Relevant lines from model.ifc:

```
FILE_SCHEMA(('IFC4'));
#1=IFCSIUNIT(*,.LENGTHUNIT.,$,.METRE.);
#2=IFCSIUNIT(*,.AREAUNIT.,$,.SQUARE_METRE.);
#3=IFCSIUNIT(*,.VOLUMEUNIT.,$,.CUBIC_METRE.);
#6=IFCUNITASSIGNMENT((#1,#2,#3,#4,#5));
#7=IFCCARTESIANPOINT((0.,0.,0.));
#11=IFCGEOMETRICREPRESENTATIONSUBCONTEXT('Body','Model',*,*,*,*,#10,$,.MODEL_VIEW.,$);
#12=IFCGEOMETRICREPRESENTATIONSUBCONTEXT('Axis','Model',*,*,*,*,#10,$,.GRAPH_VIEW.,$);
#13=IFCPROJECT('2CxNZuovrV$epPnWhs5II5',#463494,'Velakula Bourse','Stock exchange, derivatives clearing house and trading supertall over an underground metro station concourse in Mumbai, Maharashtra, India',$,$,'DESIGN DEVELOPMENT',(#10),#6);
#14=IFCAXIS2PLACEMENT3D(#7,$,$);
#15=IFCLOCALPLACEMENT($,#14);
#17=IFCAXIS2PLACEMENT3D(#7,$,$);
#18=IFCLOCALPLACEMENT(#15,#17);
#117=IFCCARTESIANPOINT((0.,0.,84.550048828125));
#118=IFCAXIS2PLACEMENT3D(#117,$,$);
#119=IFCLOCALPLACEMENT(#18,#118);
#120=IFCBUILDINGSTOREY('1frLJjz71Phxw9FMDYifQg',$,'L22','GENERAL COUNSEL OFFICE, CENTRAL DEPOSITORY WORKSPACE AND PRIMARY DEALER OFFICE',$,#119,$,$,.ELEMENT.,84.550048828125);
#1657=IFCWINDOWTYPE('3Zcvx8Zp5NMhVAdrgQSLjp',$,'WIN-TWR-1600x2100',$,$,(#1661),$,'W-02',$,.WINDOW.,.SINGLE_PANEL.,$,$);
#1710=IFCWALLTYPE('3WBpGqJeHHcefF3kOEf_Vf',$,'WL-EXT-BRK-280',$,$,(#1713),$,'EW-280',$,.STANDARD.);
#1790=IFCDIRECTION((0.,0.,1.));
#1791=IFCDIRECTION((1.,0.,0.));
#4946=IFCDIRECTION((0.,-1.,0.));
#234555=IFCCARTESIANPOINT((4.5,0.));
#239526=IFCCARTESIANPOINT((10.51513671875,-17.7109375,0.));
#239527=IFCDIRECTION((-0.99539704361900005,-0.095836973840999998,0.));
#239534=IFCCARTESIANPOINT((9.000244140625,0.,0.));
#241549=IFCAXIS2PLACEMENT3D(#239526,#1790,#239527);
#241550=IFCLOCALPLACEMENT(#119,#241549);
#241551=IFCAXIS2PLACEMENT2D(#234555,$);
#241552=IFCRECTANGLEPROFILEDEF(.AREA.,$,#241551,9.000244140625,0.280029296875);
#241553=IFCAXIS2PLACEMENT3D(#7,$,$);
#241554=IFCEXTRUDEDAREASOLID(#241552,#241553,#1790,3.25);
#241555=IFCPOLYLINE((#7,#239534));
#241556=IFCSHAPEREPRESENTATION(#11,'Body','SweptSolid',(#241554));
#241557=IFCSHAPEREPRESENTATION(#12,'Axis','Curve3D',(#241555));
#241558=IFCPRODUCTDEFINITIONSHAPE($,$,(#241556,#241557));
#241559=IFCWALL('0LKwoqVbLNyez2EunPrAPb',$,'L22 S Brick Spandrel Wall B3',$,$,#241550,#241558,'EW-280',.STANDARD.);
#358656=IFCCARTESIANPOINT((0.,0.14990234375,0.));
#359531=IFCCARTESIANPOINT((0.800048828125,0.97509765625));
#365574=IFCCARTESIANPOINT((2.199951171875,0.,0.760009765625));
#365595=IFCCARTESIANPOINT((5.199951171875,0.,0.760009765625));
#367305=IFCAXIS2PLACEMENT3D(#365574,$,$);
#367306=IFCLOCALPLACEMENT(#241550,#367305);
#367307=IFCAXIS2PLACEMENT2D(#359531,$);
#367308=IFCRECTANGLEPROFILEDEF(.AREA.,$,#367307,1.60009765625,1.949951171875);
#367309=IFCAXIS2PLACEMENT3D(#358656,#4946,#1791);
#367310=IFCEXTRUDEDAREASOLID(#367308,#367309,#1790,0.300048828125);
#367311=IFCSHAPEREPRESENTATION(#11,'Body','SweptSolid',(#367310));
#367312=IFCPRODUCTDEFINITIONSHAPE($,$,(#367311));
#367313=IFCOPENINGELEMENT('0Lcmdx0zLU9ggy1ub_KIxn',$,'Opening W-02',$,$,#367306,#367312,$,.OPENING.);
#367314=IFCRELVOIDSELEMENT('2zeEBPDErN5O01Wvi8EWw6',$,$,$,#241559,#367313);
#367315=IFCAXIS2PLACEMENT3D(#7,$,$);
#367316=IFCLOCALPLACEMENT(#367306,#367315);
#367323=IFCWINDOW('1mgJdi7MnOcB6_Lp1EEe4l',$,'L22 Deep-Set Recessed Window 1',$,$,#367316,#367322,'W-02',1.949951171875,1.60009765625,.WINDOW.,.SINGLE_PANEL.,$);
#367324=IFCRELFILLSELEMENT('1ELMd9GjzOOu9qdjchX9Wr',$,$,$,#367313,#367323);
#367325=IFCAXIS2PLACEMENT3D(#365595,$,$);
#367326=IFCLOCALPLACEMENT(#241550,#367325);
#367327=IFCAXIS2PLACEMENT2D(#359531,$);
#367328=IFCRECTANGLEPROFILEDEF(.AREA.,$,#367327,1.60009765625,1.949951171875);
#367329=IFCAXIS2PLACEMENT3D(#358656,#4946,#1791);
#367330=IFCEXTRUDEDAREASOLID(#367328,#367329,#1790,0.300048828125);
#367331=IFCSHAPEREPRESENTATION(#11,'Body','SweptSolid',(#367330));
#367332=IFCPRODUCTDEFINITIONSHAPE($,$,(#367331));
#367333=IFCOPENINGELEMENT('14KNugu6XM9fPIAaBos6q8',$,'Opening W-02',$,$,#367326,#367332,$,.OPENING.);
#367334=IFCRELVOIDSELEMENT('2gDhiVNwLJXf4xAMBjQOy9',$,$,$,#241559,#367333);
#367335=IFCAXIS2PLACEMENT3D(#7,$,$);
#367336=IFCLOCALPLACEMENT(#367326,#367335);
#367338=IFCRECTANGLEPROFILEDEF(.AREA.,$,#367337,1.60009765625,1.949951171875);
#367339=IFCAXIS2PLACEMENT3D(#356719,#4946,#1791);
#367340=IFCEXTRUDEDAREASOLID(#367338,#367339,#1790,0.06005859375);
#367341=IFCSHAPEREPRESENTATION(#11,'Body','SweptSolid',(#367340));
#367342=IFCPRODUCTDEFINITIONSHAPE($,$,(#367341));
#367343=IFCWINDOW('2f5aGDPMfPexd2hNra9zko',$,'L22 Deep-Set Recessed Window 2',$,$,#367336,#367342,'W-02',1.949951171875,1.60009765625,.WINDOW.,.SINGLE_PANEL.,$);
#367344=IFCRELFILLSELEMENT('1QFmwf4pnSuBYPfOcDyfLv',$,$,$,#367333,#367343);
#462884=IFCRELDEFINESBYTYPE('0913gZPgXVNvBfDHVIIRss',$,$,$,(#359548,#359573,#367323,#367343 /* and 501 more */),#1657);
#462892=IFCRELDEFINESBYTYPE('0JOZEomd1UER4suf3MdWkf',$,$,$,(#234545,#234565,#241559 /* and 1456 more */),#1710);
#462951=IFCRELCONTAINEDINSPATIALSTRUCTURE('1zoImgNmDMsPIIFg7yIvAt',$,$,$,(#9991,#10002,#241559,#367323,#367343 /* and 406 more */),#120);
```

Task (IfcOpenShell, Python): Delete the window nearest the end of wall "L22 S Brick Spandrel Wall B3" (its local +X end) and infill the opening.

```python
import ifcopenshell
import ifcopenshell.api.feature
import ifcopenshell.api.root
import ifcopenshell.geom
import ifcopenshell.util.shape

model = ifcopenshell.open("model.ifc")
settings = ifcopenshell.geom.settings()


def volume(element):
    """Net volume in cubic metres, openings subtracted."""
    shape = ifcopenshell.geom.create_shape(settings, element)
    return ifcopenshell.util.shape.get_volume(shape.geometry)


window = model.by_guid("2f5aGDPMfPexd2hNra9zko")
opening = window.FillsVoids[0].RelatingOpeningElement
wall = opening.VoidsElements[0].RelatingBuildingElement
before = volume(wall)

ifcopenshell.api.root.remove_product(model, product=window)
ifcopenshell.api.feature.remove_feature(model, feature=opening)

after = volume(wall)

print(f"wall volume {before:.3f} -> {after:.3f} m3")

model.write("model_v2.ifc")
```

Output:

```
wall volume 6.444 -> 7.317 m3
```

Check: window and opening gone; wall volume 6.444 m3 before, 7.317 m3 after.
